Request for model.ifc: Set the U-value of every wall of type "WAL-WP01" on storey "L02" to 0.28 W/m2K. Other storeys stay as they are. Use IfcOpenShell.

First a look at what the model holds.

```python
import ifcopenshell
import ifcopenshell.util.element

model = ifcopenshell.open("model.ifc")
print(model.schema)
storey = next(s for s in model.by_type("IfcBuildingStorey") if s.Name == "L02")
walls = [e for e in ifcopenshell.util.element.get_decomposition(storey) if e.is_a("IfcWall")]
seen = {}
for e in walls:
    element_type = ifcopenshell.util.element.get_type(e)
    key = (element_type.Name if element_type != e and element_type else None, ifcopenshell.util.element.get_pset(e, "Pset_WallCommon", "ThermalTransmittance"))
    seen[key] = seen.get(key, 0) + 1
for (name, value), count in sorted(seen.items(), key=str):
    print(count, "x", name, "|", value)
```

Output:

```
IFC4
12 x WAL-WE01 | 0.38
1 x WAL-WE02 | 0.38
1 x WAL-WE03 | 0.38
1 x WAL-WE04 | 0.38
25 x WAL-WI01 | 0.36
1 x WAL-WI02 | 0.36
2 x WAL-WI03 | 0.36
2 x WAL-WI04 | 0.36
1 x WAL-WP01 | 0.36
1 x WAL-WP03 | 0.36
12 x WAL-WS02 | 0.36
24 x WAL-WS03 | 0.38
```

```python
import ifcopenshell
import ifcopenshell.api.pset
import ifcopenshell.util.element

model = ifcopenshell.open("model.ifc")

storey = next(s for s in model.by_type("IfcBuildingStorey") if s.Name == "L02")
walls = [e for e in ifcopenshell.util.element.get_decomposition(storey) if e.is_a("IfcWall")]

count = 0
for e in walls:
    element_type = ifcopenshell.util.element.get_type(e)
    if element_type in (None, e) or element_type.Name != "WAL-WP01":
        continue
    # add_pset returns the element's existing set when there is one.
    pset = ifcopenshell.api.pset.add_pset(model, product=e, name="Pset_WallCommon")
    ifcopenshell.api.pset.edit_pset(model, pset=pset, properties={"ThermalTransmittance": 0.28})
    count += 1

print(count, "walls updated")

model.write("model_updated.ifc")
```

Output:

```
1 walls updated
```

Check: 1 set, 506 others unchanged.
